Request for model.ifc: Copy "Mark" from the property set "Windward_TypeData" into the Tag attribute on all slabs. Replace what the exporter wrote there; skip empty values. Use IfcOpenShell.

First a look at what the model holds.

```python
import ifcopenshell
import ifcopenshell.util.element

model = ifcopenshell.open("model.ifc")
print(model.schema)
slabs = model.by_type("IfcSlab")
print(len(slabs), "slabs")
for e in slabs[:8]:
    source = ifcopenshell.util.element.get_pset(e, "Windward_TypeData", "Mark")
    target = e.Tag
    print(e.id(), repr(source), repr(target), sep=" | ")
```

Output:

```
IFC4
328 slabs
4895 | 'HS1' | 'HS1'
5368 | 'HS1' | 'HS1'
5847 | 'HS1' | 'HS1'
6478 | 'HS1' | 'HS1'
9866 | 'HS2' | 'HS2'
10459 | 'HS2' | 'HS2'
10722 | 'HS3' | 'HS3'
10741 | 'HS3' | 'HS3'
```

```python
import ifcopenshell
import ifcopenshell.util.element

model = ifcopenshell.open("model.ifc")

count = 0
for e in model.by_type("IfcSlab"):
    value = ifcopenshell.util.element.get_pset(e, "Windward_TypeData", "Mark")
    current = e.Tag
    if not value or not value.strip() or current == value:
        continue
    e.Tag = value
    count += 1

print(count, "slabs updated")

model.write("model_updated.ifc")
```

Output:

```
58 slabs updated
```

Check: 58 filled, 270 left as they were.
